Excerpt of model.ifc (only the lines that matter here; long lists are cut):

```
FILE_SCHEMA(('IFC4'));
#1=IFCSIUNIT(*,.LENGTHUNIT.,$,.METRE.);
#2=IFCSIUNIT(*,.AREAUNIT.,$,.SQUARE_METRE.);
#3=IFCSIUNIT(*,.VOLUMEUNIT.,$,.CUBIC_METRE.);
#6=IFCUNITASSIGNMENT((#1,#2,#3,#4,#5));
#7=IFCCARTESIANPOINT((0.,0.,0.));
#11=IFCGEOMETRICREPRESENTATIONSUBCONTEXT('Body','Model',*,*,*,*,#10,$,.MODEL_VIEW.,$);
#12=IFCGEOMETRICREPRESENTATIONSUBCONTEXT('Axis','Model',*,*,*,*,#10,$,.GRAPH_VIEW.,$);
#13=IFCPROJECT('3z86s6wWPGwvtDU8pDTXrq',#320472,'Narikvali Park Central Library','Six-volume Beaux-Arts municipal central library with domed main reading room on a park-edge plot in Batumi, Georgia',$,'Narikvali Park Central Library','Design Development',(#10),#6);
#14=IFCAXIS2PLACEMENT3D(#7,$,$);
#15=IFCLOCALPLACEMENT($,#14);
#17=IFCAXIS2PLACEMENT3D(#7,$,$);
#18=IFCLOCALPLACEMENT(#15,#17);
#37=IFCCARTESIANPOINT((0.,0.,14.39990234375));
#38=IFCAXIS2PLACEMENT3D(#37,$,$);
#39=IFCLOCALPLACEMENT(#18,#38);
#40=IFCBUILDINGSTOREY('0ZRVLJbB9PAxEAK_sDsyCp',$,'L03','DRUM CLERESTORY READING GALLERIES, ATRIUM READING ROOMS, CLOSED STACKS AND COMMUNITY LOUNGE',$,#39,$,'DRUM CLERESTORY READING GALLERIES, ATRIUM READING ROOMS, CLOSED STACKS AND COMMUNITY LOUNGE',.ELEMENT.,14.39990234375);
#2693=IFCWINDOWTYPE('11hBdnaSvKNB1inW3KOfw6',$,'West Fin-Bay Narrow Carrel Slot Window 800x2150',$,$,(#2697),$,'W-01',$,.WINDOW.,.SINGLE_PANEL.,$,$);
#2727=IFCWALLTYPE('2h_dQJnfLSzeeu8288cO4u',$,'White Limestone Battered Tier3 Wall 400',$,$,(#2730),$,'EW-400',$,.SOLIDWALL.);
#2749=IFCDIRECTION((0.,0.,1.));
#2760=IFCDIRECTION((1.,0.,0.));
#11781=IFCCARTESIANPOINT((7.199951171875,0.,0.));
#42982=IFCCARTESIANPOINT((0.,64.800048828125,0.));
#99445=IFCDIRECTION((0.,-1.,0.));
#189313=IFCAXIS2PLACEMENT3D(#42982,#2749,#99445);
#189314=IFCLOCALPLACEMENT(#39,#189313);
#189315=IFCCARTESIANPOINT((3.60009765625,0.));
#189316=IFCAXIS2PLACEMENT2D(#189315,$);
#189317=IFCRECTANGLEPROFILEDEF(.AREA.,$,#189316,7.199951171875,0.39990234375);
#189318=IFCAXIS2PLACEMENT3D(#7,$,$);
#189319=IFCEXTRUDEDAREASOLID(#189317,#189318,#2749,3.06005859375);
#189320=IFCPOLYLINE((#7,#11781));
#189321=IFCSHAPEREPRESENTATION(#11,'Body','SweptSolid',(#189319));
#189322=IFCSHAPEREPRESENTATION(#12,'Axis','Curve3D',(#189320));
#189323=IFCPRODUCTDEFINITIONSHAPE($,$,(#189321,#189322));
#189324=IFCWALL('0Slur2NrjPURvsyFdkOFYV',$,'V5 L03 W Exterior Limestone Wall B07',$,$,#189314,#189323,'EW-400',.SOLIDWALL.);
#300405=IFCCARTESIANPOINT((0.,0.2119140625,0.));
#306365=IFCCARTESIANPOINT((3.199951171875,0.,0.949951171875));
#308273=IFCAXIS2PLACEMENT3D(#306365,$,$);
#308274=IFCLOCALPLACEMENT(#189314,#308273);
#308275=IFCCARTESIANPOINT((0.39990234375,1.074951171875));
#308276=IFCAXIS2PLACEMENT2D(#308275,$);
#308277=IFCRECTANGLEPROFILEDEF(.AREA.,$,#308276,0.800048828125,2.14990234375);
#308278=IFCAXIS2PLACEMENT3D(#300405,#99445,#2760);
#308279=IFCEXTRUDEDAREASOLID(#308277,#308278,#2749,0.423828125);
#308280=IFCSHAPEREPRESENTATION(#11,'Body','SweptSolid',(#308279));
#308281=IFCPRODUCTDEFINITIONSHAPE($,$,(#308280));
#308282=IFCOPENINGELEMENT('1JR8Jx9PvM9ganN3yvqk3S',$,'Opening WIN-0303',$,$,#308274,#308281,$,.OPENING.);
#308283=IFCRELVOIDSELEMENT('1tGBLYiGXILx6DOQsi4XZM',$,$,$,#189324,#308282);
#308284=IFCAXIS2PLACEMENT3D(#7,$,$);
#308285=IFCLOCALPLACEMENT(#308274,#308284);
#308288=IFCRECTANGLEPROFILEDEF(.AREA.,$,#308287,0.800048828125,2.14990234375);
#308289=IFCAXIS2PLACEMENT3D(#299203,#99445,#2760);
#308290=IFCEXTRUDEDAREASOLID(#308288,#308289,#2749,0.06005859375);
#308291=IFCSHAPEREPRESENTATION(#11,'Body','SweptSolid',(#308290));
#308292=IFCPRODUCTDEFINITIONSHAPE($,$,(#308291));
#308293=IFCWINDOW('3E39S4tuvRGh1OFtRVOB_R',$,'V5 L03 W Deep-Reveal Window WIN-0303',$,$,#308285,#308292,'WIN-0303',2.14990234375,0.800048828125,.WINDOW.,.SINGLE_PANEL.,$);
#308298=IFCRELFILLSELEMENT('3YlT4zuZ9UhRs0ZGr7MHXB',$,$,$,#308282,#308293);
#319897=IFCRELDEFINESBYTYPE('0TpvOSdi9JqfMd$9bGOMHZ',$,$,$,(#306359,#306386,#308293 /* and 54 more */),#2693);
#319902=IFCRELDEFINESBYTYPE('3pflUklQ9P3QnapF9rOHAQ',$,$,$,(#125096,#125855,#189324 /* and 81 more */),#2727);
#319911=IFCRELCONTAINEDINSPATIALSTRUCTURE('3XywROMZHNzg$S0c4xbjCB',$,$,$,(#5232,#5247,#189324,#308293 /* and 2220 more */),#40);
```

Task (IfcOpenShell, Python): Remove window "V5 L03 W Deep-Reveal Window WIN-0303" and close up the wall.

```python
import ifcopenshell
import ifcopenshell.api.feature
import ifcopenshell.api.root
import ifcopenshell.geom
import ifcopenshell.util.shape

model = ifcopenshell.open("model.ifc")
settings = ifcopenshell.geom.settings()


def volume(element):
    """Net volume in cubic metres, openings subtracted."""
    shape = ifcopenshell.geom.create_shape(settings, element)
    return ifcopenshell.util.shape.get_volume(shape.geometry)


window = model.by_guid("3E39S4tuvRGh1OFtRVOB_R")
opening = window.FillsVoids[0].RelatingOpeningElement
wall = opening.VoidsElements[0].RelatingBuildingElement
before = volume(wall)

ifcopenshell.api.root.remove_product(model, product=window)
ifcopenshell.api.feature.remove_feature(model, feature=opening)

after = volume(wall)

print(f"wall volume {before:.3f} -> {after:.3f} m3")

model.write("model_rev.ifc")
```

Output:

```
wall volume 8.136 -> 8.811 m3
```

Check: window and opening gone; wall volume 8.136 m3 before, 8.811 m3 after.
